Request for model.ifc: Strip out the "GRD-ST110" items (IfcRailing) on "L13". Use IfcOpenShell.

First a look at what the model holds.

```python
import ifcopenshell
import ifcopenshell.util.element

model = ifcopenshell.open("model.ifc")
print(model.schema)
storey = next(s for s in model.by_type("IfcBuildingStorey") if s.Name == "L13")
railings = [e for e in ifcopenshell.util.element.get_decomposition(storey) if e.is_a("IfcRailing")]
seen = {}
for e in railings:
    element_type = ifcopenshell.util.element.get_type(e)
    name = element_type.Name if element_type not in (None, e) else None
    seen[name] = seen.get(name, 0) + 1
for name, count in sorted(seen.items(), key=str):
    print(count, "x", name)
```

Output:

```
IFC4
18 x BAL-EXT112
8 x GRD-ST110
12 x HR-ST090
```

```python
import ifcopenshell
import ifcopenshell.api.root
import ifcopenshell.util.element

model = ifcopenshell.open("model.ifc")

storey = next(s for s in model.by_type("IfcBuildingStorey") if s.Name == "L13")
railings = [e for e in ifcopenshell.util.element.get_decomposition(storey) if e.is_a("IfcRailing")]
targets = [e for e in railings if (t := ifcopenshell.util.element.get_type(e)) not in (None, e) and t.Name == "GRD-ST110"]

for e in targets:
    ifcopenshell.api.root.remove_product(model, product=e)
print(len(targets), "removed")

model.write("model_rev.ifc")
```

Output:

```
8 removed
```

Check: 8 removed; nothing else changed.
